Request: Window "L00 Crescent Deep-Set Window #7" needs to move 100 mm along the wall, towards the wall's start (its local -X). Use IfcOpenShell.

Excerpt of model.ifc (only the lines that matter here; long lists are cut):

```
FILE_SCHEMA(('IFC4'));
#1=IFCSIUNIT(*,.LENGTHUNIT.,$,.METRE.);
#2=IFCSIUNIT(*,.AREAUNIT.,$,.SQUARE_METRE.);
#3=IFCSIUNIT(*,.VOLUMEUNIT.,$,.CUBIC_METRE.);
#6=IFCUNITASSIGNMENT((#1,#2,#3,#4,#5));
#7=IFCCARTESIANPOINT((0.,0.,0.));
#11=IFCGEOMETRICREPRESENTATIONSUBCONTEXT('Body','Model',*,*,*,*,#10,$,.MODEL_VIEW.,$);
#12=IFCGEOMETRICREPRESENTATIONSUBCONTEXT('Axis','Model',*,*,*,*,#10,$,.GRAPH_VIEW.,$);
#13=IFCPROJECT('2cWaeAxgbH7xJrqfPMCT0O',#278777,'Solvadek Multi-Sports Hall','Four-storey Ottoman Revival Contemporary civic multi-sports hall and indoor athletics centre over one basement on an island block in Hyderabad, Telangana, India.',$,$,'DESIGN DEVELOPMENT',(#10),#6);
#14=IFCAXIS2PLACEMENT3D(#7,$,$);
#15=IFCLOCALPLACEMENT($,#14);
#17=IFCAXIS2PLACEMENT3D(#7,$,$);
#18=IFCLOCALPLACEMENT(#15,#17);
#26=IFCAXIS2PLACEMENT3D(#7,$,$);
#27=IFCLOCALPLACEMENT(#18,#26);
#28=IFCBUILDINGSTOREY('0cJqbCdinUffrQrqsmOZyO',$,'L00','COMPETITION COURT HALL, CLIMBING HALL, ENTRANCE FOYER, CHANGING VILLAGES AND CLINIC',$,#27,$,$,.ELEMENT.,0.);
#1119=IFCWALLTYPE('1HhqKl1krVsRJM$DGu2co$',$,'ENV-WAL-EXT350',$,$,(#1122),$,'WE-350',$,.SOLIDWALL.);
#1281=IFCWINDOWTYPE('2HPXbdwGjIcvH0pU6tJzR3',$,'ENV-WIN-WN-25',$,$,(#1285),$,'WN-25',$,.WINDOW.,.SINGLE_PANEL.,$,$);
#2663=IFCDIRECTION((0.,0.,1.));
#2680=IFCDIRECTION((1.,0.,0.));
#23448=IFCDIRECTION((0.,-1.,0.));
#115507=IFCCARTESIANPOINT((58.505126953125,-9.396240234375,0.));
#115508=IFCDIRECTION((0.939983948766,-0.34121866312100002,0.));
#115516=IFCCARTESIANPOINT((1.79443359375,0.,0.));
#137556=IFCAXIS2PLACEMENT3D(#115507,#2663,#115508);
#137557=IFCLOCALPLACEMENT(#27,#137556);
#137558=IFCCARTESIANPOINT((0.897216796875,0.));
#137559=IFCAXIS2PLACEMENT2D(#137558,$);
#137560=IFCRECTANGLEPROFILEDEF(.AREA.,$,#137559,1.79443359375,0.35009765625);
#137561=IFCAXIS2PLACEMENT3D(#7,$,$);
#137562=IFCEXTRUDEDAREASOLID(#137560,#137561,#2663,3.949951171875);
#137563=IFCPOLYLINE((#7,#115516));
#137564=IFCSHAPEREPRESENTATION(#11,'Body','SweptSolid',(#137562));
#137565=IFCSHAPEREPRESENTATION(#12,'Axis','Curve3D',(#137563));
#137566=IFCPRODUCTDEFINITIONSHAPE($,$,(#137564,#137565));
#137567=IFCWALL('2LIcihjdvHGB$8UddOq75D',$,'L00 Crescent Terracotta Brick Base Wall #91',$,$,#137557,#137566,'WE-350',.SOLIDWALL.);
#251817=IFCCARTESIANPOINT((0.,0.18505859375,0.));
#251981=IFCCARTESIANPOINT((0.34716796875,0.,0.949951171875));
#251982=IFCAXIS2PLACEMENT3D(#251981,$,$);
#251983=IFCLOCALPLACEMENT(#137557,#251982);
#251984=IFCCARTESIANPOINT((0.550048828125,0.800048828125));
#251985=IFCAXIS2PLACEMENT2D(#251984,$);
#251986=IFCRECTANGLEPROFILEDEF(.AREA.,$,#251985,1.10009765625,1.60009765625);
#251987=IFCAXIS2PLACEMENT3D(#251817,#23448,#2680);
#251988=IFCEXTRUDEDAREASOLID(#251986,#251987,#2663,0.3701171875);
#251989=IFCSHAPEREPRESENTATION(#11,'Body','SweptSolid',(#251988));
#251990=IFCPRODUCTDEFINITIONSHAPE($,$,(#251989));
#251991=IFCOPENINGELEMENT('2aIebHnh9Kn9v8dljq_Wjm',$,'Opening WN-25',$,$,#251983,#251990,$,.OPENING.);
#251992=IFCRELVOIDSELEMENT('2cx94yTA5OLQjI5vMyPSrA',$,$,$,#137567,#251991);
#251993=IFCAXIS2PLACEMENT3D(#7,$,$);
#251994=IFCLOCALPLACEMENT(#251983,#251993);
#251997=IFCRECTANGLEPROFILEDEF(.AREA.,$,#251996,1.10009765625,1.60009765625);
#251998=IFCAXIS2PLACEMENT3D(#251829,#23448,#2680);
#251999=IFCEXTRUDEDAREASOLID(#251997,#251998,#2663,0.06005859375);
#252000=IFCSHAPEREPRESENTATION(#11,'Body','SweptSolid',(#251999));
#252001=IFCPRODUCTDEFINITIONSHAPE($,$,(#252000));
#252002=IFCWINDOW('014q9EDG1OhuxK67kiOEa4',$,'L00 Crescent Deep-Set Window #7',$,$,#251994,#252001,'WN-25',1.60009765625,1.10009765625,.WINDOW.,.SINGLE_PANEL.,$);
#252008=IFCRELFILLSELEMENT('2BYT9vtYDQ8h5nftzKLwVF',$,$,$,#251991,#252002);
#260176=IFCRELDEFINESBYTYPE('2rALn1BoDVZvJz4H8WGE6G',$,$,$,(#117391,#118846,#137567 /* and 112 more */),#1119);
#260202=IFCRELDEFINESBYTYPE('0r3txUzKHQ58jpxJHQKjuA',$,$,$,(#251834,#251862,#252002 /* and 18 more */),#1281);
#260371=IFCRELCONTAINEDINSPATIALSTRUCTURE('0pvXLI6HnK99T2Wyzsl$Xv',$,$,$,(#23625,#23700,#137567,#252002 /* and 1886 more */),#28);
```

```python
import ifcopenshell
import ifcopenshell.api.geometry
import ifcopenshell.util.placement
import ifcopenshell.util.unit

model = ifcopenshell.open("model.ifc")
unit_scale = ifcopenshell.util.unit.calculate_unit_scale(model)

window = model.by_guid("014q9EDG1OhuxK67kiOEa4")
opening = window.FillsVoids[0].RelatingOpeningElement
wall = opening.VoidsElements[0].RelatingBuildingElement

wall_matrix = ifcopenshell.util.placement.get_local_placement(wall.ObjectPlacement)
shift = wall_matrix[:3, 0] * -0.1 / unit_scale
before = ifcopenshell.util.placement.get_local_placement(window.ObjectPlacement)[:3, 3].copy()

# The window is placed relative to its opening, so it follows when the opening moves.
matrix = ifcopenshell.util.placement.get_local_placement(opening.ObjectPlacement)
matrix[:3, 3] += shift
ifcopenshell.api.geometry.edit_object_placement(
    model, product=opening, matrix=matrix, is_si=False, should_transform_children=True
)

after = ifcopenshell.util.placement.get_local_placement(window.ObjectPlacement)[:3, 3]
print("window moved by", (after - before).round(3) + 0.0)

model.write("model_v2.ifc")
```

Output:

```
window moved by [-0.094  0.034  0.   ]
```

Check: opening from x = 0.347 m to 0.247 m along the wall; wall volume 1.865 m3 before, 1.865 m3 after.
